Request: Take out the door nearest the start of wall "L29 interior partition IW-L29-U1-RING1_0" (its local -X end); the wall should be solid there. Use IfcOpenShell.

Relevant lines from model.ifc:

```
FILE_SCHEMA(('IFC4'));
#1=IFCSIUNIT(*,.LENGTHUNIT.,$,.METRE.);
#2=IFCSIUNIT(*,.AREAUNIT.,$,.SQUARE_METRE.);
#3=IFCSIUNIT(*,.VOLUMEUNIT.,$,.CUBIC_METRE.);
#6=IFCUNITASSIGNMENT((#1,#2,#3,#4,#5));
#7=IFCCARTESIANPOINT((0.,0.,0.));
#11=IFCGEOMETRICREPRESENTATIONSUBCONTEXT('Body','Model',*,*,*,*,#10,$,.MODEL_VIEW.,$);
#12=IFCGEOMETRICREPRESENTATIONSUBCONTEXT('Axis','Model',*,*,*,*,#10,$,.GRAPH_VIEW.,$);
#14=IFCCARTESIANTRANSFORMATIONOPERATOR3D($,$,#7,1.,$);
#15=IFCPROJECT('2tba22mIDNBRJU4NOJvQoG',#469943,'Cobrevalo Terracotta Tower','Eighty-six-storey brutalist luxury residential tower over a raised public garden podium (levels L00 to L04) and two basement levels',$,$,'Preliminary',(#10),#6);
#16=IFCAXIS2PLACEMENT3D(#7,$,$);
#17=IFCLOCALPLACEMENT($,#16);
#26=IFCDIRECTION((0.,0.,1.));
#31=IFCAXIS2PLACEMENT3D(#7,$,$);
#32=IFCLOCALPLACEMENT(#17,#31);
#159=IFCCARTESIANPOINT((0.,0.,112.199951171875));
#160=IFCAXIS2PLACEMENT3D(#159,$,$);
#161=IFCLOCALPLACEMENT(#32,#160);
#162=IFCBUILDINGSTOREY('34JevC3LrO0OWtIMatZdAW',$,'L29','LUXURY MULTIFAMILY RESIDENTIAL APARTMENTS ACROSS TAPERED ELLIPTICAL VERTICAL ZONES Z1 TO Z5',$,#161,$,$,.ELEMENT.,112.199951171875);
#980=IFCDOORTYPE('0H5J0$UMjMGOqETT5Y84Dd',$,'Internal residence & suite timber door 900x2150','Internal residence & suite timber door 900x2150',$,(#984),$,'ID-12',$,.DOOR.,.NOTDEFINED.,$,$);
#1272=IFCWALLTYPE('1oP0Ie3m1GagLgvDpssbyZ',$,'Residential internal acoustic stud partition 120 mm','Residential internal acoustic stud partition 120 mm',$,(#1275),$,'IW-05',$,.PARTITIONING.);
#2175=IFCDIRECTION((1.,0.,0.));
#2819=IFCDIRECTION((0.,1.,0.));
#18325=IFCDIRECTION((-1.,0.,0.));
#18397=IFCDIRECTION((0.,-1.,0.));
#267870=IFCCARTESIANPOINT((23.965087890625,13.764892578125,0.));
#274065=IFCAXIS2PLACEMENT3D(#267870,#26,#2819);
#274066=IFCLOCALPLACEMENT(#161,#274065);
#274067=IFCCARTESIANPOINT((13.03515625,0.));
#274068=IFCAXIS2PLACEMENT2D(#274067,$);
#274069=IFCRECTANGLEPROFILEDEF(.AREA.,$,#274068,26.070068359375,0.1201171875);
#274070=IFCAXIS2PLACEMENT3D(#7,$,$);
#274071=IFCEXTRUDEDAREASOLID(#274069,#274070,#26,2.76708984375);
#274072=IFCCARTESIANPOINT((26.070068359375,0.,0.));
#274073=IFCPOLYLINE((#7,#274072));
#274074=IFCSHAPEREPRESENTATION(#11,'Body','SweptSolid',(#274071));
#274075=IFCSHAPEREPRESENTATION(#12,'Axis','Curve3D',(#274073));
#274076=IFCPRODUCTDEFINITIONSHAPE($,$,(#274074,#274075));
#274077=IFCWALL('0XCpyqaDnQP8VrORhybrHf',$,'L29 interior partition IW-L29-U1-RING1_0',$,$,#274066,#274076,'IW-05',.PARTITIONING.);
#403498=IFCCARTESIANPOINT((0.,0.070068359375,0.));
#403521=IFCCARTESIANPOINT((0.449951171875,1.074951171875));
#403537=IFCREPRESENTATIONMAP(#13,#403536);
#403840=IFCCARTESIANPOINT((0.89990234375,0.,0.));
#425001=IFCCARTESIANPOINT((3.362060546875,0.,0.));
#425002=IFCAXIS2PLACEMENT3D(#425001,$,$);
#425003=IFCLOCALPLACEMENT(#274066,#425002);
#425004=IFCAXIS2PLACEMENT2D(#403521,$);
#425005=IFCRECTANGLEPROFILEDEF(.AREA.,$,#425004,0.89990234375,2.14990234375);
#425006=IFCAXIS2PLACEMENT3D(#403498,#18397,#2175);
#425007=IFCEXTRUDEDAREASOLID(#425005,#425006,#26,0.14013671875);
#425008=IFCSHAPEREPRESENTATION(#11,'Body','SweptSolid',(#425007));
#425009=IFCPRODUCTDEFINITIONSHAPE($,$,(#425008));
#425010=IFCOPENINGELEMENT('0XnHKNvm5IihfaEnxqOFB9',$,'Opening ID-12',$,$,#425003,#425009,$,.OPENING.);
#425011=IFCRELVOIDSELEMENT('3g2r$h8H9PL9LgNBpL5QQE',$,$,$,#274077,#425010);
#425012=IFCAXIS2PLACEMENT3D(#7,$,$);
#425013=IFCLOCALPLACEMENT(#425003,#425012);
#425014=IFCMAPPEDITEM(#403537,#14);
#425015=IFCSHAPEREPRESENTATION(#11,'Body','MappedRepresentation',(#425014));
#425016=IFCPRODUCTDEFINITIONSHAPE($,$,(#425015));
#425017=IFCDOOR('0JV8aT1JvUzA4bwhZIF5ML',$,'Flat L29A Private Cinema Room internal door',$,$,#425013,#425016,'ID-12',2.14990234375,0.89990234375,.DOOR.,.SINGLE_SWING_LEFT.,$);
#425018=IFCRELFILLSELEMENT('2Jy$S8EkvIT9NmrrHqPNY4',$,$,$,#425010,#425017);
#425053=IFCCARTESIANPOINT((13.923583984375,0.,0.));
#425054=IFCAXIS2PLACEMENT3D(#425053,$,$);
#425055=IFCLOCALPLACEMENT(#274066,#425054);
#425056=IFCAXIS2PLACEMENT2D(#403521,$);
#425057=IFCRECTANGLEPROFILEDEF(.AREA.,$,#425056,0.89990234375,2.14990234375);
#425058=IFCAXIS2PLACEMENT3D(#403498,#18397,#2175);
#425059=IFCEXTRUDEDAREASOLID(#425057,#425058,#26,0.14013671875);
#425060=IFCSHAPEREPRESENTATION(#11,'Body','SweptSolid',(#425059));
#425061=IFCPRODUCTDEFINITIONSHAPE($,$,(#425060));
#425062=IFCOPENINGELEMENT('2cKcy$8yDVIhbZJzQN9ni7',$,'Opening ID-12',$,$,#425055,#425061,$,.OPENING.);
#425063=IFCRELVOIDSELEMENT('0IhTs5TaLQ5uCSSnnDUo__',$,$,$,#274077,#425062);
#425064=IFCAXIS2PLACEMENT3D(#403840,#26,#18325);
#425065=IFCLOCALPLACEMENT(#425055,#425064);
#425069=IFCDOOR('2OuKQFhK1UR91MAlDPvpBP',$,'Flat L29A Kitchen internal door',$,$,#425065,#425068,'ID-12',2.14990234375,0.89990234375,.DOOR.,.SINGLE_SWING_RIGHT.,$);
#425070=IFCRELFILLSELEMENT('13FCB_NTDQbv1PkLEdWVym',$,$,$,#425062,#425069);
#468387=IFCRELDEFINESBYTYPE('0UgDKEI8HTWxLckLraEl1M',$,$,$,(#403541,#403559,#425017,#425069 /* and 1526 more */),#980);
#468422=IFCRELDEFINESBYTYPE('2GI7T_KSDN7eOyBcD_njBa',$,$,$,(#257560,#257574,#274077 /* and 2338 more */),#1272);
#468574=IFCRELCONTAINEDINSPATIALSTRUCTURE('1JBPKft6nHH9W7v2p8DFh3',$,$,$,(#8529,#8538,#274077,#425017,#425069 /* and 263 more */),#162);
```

```python
import ifcopenshell
import ifcopenshell.api.feature
import ifcopenshell.api.root
import ifcopenshell.geom
import ifcopenshell.util.shape

model = ifcopenshell.open("model.ifc")
settings = ifcopenshell.geom.settings()


def volume(element):
    """Net volume in cubic metres, openings subtracted."""
    shape = ifcopenshell.geom.create_shape(settings, element)
    return ifcopenshell.util.shape.get_volume(shape.geometry)


door = model.by_guid("0JV8aT1JvUzA4bwhZIF5ML")
opening = door.FillsVoids[0].RelatingOpeningElement
wall = opening.VoidsElements[0].RelatingBuildingElement
before = volume(wall)

ifcopenshell.api.root.remove_product(model, product=door)
ifcopenshell.api.feature.remove_feature(model, feature=opening)

after = volume(wall)

print(f"wall volume {before:.3f} -> {after:.3f} m3")

model.write("model-out.ifc")
```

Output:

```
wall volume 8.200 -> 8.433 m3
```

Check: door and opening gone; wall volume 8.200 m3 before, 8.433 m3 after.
